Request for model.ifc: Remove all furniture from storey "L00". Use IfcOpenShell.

First a look at what the model holds.

```python
import ifcopenshell
import ifcopenshell.util.element

model = ifcopenshell.open("model.ifc")
print(model.schema)
storey = next(s for s in model.by_type("IfcBuildingStorey") if s.Name == "L00")
furniture = [e for e in ifcopenshell.util.element.get_decomposition(storey) if e.is_a("IfcFurnishingElement")]
seen = {}
for e in furniture:
    element_type = ifcopenshell.util.element.get_type(e)
    name = element_type.Name if element_type not in (None, e) else None
    seen[name] = seen.get(name, 0) + 1
for name, count in sorted(seen.items(), key=str):
    print(count, "x", name)
```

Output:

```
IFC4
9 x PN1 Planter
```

```python
import ifcopenshell
import ifcopenshell.api.root
import ifcopenshell.util.element

model = ifcopenshell.open("model.ifc")

storey = next(s for s in model.by_type("IfcBuildingStorey") if s.Name == "L00")
furniture = [e for e in ifcopenshell.util.element.get_decomposition(storey) if e.is_a("IfcFurnishingElement")]

for e in furniture:
    ifcopenshell.api.root.remove_product(model, product=e)
print(len(furniture), "removed")

model.write("model_edited.ifc")
```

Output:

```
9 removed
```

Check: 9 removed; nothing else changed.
